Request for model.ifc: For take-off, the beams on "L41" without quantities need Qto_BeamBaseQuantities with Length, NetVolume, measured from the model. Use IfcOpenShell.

First a look at what the model holds.

```python
import ifcopenshell
import ifcopenshell.util.element
import ifcopenshell.util.unit

model = ifcopenshell.open("model.ifc")
print(model.schema)
for unit_type in ("LENGTHUNIT", "AREAUNIT", "VOLUMEUNIT"):
    print(unit_type, ifcopenshell.util.unit.calculate_unit_scale(model, unit_type))
storey = next(s for s in model.by_type("IfcBuildingStorey") if s.Name == "L41")
beams = [e for e in ifcopenshell.util.element.get_decomposition(storey) if e.is_a("IfcBeam")]
for e in sorted(beams, key=lambda e: e.id()):
    print(e.id(), e.is_a(), e.Name, list(ifcopenshell.util.element.get_psets(e, qtos_only=True)), sep=" | ")
```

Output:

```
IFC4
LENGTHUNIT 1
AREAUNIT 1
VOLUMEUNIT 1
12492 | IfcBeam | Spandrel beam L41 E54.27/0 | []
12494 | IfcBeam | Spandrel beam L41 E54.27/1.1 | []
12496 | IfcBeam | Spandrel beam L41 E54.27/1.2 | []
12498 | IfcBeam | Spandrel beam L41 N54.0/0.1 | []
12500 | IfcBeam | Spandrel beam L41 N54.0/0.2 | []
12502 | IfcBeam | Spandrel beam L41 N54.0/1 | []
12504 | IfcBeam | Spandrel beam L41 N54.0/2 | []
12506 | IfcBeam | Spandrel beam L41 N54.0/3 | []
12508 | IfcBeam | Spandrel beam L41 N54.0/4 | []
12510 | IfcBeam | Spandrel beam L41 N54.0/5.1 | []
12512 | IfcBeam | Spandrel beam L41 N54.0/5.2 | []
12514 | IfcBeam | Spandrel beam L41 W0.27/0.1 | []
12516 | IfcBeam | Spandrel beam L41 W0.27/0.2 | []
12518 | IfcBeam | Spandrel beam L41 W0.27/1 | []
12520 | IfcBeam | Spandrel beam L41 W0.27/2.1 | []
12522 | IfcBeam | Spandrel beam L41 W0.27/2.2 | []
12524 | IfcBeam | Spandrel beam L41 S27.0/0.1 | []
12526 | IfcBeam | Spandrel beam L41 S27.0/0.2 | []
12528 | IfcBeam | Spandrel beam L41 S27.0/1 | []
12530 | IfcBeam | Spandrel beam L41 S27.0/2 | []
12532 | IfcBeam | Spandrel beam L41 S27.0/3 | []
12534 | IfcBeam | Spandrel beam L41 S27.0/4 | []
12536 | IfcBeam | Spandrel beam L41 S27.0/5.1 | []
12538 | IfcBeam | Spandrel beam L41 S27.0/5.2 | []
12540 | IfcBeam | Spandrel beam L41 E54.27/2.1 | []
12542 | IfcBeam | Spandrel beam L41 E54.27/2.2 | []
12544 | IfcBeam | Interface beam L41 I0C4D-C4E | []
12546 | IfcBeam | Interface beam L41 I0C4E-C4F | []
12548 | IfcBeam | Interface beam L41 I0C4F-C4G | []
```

```python
import ifcopenshell
import ifcopenshell.api.pset
import ifcopenshell.geom
import ifcopenshell.util.element
import ifcopenshell.util.shape
import ifcopenshell.util.unit

model = ifcopenshell.open("model.ifc")
unit_scale = ifcopenshell.util.unit.calculate_unit_scale(model)
volume_scale = ifcopenshell.util.unit.calculate_unit_scale(model, "VOLUMEUNIT")
settings = ifcopenshell.geom.settings()

storey = next(s for s in model.by_type("IfcBuildingStorey") if s.Name == "L41")
beams = [e for e in ifcopenshell.util.element.get_decomposition(storey) if e.is_a("IfcBeam")]

for e in sorted(beams, key=lambda e: e.id()):
    if ifcopenshell.util.element.get_psets(e, qtos_only=True, should_inherit=False):
        continue
    # Geometry comes back in metres, in the element's own axes.
    shape = ifcopenshell.geom.create_shape(settings, e)
    values = {
        "Length": ifcopenshell.util.shape.get_max_xyz(shape.geometry) / unit_scale,
        "NetVolume": ifcopenshell.util.shape.get_volume(shape.geometry) / volume_scale,
    }
    qto = ifcopenshell.api.pset.add_qto(model, product=e, name="Qto_BeamBaseQuantities")
    ifcopenshell.api.pset.edit_qto(model, qto=qto, properties=values)
    print(e.id(), {k: round(v, 3) for k, v in values.items()})

model.write("model_edited.ifc")
```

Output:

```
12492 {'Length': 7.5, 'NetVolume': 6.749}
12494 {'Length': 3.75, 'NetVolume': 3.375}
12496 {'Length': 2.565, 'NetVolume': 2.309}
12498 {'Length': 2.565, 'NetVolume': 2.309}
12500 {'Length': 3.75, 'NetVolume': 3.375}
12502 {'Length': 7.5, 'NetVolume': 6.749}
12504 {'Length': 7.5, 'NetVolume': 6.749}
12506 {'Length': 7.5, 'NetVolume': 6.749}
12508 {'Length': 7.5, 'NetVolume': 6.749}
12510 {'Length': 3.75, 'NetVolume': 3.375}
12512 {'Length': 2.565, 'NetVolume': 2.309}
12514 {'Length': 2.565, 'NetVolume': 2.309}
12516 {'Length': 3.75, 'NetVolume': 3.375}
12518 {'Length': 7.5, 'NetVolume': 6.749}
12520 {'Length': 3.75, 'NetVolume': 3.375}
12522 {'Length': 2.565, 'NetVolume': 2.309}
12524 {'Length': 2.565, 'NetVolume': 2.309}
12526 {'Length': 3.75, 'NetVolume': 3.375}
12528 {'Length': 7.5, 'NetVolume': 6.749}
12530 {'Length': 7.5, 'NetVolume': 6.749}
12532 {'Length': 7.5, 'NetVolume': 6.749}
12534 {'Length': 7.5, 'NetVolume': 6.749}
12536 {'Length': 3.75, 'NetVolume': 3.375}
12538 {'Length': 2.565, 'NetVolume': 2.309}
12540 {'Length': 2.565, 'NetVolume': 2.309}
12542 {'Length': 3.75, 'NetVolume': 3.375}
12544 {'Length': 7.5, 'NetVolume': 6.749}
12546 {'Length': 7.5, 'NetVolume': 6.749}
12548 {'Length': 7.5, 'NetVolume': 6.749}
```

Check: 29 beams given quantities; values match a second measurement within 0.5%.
